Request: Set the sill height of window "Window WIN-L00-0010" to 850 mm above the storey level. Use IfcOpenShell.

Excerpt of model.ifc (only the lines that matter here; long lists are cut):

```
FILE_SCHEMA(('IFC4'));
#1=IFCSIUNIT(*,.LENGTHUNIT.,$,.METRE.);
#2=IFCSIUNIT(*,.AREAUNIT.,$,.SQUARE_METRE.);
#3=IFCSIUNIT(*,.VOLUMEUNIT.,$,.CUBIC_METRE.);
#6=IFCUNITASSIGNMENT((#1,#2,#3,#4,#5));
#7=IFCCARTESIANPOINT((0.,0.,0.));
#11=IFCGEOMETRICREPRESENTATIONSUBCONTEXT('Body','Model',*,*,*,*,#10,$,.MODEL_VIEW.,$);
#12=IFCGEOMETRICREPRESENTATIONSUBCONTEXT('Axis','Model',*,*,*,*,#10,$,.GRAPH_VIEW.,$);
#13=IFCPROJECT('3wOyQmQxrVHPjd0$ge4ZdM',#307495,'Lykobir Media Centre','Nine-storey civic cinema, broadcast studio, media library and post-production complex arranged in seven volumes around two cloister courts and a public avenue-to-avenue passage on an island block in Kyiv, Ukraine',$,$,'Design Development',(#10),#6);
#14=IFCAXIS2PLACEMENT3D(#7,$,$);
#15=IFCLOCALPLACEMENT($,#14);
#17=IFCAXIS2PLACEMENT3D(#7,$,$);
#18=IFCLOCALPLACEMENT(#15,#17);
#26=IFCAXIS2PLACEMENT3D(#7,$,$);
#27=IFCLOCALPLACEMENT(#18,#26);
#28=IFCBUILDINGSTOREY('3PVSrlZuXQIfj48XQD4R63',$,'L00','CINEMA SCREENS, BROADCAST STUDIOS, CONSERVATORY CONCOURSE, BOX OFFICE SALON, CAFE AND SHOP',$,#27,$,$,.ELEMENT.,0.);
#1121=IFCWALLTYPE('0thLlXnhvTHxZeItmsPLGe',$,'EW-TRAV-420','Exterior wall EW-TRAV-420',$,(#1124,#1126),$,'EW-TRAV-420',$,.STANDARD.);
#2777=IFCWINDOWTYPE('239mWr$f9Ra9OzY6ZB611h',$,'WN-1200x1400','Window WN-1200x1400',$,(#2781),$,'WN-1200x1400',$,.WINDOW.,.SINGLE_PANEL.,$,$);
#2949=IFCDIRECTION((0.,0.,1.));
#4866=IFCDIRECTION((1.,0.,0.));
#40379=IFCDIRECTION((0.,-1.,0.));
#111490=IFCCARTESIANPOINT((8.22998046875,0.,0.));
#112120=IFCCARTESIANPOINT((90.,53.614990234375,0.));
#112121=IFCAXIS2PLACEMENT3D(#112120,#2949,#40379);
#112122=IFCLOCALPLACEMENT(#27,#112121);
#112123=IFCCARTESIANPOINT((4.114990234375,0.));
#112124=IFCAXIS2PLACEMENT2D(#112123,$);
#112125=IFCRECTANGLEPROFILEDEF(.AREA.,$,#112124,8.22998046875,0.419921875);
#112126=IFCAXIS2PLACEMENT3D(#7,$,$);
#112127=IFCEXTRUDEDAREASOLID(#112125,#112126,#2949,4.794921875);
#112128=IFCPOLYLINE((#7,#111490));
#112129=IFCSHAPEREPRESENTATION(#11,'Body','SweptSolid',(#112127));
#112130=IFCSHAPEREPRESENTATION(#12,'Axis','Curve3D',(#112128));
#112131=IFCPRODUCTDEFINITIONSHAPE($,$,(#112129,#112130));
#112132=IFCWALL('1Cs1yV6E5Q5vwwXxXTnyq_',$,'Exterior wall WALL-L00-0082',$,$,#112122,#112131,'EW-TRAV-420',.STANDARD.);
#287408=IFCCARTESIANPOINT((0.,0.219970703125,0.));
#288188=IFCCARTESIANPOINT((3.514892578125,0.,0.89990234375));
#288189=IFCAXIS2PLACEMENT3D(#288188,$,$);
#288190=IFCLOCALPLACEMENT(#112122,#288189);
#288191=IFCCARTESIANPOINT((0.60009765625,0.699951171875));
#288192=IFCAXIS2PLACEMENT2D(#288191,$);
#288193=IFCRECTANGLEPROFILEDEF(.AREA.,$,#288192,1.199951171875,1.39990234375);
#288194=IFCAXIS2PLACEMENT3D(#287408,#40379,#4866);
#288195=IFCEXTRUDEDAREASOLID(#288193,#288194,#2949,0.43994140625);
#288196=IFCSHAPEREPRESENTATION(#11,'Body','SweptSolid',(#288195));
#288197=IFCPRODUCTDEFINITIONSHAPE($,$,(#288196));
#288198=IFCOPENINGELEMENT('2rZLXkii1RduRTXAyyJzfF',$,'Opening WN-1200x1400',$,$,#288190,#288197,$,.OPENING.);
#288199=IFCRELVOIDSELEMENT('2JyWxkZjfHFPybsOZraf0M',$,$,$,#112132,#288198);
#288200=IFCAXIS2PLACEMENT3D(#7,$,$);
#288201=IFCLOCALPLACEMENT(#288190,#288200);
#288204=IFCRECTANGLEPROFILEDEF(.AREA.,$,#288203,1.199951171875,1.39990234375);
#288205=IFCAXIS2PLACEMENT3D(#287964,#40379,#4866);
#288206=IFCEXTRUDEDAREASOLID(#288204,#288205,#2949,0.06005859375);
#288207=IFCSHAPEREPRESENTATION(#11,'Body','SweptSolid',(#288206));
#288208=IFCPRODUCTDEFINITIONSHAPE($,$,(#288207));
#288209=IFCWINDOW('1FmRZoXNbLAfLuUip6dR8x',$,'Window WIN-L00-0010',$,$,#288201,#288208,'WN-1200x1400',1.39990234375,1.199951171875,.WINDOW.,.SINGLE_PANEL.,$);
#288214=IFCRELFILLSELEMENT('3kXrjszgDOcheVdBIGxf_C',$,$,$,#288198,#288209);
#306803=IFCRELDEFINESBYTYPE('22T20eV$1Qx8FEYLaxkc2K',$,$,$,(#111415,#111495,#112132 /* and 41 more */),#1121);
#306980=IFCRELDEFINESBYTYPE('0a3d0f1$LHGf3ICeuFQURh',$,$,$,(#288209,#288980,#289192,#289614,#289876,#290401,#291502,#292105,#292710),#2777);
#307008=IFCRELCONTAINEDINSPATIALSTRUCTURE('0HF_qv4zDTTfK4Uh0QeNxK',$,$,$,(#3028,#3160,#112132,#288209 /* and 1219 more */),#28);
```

```python
import numpy as np
import ifcopenshell
import ifcopenshell.api.geometry
import ifcopenshell.geom
import ifcopenshell.util.element
import ifcopenshell.util.placement
import ifcopenshell.util.shape
import ifcopenshell.util.unit

model = ifcopenshell.open("model.ifc")
unit_scale = ifcopenshell.util.unit.calculate_unit_scale(model)

window = model.by_id(288209)
opening = window.FillsVoids[0].RelatingOpeningElement
storey = ifcopenshell.util.element.get_container(window, ifc_class="IfcBuildingStorey")
level = ifcopenshell.util.placement.get_local_placement(storey.ObjectPlacement)[2, 3]

# The opening's origin need not be at the sill, so measure its lowest point.
shape = ifcopenshell.geom.create_shape(ifcopenshell.geom.settings(), opening)
bottom = ifcopenshell.util.shape.get_shape_bottom_elevation(shape, shape.geometry) / unit_scale
dz = level + 0.85 - bottom

shift = np.array([0.0, 0.0, dz])
# The window is placed relative to its opening, so it follows when the opening moves.
matrix = ifcopenshell.util.placement.get_local_placement(opening.ObjectPlacement)
matrix[:3, 3] += shift
ifcopenshell.api.geometry.edit_object_placement(
    model, product=opening, matrix=matrix, is_si=False, should_transform_children=True
)

print(f"moved by {dz * unit_scale:+.3f} m")

model.write("model_edited.ifc")
```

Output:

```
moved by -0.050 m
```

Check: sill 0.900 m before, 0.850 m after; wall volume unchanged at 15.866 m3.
